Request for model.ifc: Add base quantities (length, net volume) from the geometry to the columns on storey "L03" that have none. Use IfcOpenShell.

First a look at what the model holds.

```python
import ifcopenshell
import ifcopenshell.util.element
import ifcopenshell.util.unit

model = ifcopenshell.open("model.ifc")
print(model.schema)
for unit_type in ("LENGTHUNIT", "AREAUNIT", "VOLUMEUNIT"):
    print(unit_type, ifcopenshell.util.unit.calculate_unit_scale(model, unit_type))
storey = next(s for s in model.by_type("IfcBuildingStorey") if s.Name == "L03")
columns = [e for e in ifcopenshell.util.element.get_decomposition(storey) if e.is_a("IfcColumn")]
for e in sorted(columns, key=lambda e: e.id()):
    print(e.id(), e.is_a(), e.Name, list(ifcopenshell.util.element.get_psets(e, qtos_only=True)), sep=" | ")
```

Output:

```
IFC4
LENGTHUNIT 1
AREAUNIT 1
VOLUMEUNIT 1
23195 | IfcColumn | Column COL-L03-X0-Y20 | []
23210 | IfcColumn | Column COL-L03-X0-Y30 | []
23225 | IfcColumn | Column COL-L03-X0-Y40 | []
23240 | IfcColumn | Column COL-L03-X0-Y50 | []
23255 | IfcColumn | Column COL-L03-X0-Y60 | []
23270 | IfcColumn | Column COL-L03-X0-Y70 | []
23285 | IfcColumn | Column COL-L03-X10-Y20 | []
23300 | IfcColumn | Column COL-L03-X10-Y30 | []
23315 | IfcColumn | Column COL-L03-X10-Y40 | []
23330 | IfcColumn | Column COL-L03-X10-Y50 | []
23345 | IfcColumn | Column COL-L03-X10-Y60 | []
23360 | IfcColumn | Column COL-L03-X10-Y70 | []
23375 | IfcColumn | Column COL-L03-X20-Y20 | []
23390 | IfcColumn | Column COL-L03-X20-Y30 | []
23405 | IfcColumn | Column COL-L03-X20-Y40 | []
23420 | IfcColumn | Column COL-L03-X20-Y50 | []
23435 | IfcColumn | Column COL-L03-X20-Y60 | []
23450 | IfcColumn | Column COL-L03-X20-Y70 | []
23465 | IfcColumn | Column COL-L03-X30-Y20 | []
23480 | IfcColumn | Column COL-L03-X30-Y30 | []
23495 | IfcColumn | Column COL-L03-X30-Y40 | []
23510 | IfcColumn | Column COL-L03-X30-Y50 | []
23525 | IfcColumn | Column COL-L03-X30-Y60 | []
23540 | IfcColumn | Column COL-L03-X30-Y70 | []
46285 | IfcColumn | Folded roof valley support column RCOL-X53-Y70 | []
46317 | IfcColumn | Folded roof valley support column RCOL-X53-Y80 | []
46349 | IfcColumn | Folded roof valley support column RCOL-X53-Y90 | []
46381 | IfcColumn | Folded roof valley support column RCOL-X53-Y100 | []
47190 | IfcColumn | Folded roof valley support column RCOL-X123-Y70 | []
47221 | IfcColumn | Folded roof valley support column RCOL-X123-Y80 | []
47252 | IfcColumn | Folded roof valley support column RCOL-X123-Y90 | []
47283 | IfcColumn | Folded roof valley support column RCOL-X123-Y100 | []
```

```python
import ifcopenshell
import ifcopenshell.api.pset
import ifcopenshell.geom
import ifcopenshell.util.element
import ifcopenshell.util.shape
import ifcopenshell.util.unit

model = ifcopenshell.open("model.ifc")
unit_scale = ifcopenshell.util.unit.calculate_unit_scale(model)
volume_scale = ifcopenshell.util.unit.calculate_unit_scale(model, "VOLUMEUNIT")
settings = ifcopenshell.geom.settings()

storey = next(s for s in model.by_type("IfcBuildingStorey") if s.Name == "L03")
columns = [e for e in ifcopenshell.util.element.get_decomposition(storey) if e.is_a("IfcColumn")]

for e in sorted(columns, key=lambda e: e.id()):
    if ifcopenshell.util.element.get_psets(e, qtos_only=True, should_inherit=False):
        continue
    # Geometry comes back in metres, in the element's own axes.
    shape = ifcopenshell.geom.create_shape(settings, e)
    values = {
        "Length": ifcopenshell.util.shape.get_z(shape.geometry) / unit_scale,
        "NetVolume": ifcopenshell.util.shape.get_volume(shape.geometry) / volume_scale,
    }
    qto = ifcopenshell.api.pset.add_qto(model, product=e, name="Qto_ColumnBaseQuantities")
    ifcopenshell.api.pset.edit_qto(model, qto=qto, properties=values)
    print(e.id(), {k: round(v, 3) for k, v in values.items()})

model.write("model_rev.ifc")
```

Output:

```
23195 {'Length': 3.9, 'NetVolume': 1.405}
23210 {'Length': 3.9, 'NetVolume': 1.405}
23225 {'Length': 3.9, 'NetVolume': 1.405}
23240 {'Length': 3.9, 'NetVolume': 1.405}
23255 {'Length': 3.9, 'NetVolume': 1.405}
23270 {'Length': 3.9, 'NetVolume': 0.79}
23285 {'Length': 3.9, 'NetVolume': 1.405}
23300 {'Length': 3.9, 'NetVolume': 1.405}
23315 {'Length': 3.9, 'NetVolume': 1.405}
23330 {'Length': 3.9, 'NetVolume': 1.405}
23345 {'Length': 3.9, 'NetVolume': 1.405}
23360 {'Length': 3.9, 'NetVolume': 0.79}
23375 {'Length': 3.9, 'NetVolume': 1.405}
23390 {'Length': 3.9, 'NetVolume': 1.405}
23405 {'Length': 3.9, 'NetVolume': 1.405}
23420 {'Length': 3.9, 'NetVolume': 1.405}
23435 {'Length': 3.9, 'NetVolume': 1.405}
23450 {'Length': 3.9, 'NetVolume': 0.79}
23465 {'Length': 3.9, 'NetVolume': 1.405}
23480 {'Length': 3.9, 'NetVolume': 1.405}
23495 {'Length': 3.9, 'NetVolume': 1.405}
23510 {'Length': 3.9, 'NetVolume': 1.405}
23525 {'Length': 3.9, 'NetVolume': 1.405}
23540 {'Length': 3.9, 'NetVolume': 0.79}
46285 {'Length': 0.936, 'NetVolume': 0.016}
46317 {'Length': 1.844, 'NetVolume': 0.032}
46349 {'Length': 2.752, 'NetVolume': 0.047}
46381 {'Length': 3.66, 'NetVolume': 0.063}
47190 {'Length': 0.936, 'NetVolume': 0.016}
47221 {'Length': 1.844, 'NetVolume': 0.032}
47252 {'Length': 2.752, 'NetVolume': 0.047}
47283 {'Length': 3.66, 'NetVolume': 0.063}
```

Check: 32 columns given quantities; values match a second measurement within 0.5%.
